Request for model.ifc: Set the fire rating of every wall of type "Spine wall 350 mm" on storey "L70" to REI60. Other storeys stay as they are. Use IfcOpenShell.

First a look at what the model holds.

```python
import ifcopenshell
import ifcopenshell.util.element

model = ifcopenshell.open("model.ifc")
print(model.schema)
storey = next(s for s in model.by_type("IfcBuildingStorey") if s.Name == "L70")
walls = [e for e in ifcopenshell.util.element.get_decomposition(storey) if e.is_a("IfcWall")]
seen = {}
for e in walls:
    element_type = ifcopenshell.util.element.get_type(e)
    key = (element_type.Name if element_type != e and element_type else None, ifcopenshell.util.element.get_pset(e, "Pset_WallCommon", "FireRating"))
    seen[key] = seen.get(key, 0) + 1
for (name, value), count in sorted(seen.items(), key=str):
    print(count, "x", name, "|", value)
```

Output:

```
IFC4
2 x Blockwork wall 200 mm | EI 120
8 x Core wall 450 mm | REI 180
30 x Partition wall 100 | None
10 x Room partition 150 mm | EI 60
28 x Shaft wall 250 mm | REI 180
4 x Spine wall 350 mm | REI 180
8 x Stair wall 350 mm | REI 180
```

```python
import ifcopenshell
import ifcopenshell.api.pset
import ifcopenshell.util.element

model = ifcopenshell.open("model.ifc")

storey = next(s for s in model.by_type("IfcBuildingStorey") if s.Name == "L70")
walls = [e for e in ifcopenshell.util.element.get_decomposition(storey) if e.is_a("IfcWall")]

count = 0
for e in walls:
    element_type = ifcopenshell.util.element.get_type(e)
    if element_type in (None, e) or element_type.Name != "Spine wall 350 mm":
        continue
    found = ifcopenshell.util.element.get_pset(e, "Pset_WallCommon", should_inherit=False)
    if found:
        pset = model.by_id(found["id"])
        if len(ifcopenshell.util.element.get_elements_by_pset(pset)) > 1:
            pset = ifcopenshell.api.pset.unshare_pset(model, products=[e], pset=pset)[0]
    else:
        pset = ifcopenshell.api.pset.add_pset(model, product=e, name="Pset_WallCommon")
    ifcopenshell.api.pset.edit_pset(model, pset=pset, properties={"FireRating": "REI60"})
    count += 1

print(count, "walls updated")

model.write("model_rev.ifc")
```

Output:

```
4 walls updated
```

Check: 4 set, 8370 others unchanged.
